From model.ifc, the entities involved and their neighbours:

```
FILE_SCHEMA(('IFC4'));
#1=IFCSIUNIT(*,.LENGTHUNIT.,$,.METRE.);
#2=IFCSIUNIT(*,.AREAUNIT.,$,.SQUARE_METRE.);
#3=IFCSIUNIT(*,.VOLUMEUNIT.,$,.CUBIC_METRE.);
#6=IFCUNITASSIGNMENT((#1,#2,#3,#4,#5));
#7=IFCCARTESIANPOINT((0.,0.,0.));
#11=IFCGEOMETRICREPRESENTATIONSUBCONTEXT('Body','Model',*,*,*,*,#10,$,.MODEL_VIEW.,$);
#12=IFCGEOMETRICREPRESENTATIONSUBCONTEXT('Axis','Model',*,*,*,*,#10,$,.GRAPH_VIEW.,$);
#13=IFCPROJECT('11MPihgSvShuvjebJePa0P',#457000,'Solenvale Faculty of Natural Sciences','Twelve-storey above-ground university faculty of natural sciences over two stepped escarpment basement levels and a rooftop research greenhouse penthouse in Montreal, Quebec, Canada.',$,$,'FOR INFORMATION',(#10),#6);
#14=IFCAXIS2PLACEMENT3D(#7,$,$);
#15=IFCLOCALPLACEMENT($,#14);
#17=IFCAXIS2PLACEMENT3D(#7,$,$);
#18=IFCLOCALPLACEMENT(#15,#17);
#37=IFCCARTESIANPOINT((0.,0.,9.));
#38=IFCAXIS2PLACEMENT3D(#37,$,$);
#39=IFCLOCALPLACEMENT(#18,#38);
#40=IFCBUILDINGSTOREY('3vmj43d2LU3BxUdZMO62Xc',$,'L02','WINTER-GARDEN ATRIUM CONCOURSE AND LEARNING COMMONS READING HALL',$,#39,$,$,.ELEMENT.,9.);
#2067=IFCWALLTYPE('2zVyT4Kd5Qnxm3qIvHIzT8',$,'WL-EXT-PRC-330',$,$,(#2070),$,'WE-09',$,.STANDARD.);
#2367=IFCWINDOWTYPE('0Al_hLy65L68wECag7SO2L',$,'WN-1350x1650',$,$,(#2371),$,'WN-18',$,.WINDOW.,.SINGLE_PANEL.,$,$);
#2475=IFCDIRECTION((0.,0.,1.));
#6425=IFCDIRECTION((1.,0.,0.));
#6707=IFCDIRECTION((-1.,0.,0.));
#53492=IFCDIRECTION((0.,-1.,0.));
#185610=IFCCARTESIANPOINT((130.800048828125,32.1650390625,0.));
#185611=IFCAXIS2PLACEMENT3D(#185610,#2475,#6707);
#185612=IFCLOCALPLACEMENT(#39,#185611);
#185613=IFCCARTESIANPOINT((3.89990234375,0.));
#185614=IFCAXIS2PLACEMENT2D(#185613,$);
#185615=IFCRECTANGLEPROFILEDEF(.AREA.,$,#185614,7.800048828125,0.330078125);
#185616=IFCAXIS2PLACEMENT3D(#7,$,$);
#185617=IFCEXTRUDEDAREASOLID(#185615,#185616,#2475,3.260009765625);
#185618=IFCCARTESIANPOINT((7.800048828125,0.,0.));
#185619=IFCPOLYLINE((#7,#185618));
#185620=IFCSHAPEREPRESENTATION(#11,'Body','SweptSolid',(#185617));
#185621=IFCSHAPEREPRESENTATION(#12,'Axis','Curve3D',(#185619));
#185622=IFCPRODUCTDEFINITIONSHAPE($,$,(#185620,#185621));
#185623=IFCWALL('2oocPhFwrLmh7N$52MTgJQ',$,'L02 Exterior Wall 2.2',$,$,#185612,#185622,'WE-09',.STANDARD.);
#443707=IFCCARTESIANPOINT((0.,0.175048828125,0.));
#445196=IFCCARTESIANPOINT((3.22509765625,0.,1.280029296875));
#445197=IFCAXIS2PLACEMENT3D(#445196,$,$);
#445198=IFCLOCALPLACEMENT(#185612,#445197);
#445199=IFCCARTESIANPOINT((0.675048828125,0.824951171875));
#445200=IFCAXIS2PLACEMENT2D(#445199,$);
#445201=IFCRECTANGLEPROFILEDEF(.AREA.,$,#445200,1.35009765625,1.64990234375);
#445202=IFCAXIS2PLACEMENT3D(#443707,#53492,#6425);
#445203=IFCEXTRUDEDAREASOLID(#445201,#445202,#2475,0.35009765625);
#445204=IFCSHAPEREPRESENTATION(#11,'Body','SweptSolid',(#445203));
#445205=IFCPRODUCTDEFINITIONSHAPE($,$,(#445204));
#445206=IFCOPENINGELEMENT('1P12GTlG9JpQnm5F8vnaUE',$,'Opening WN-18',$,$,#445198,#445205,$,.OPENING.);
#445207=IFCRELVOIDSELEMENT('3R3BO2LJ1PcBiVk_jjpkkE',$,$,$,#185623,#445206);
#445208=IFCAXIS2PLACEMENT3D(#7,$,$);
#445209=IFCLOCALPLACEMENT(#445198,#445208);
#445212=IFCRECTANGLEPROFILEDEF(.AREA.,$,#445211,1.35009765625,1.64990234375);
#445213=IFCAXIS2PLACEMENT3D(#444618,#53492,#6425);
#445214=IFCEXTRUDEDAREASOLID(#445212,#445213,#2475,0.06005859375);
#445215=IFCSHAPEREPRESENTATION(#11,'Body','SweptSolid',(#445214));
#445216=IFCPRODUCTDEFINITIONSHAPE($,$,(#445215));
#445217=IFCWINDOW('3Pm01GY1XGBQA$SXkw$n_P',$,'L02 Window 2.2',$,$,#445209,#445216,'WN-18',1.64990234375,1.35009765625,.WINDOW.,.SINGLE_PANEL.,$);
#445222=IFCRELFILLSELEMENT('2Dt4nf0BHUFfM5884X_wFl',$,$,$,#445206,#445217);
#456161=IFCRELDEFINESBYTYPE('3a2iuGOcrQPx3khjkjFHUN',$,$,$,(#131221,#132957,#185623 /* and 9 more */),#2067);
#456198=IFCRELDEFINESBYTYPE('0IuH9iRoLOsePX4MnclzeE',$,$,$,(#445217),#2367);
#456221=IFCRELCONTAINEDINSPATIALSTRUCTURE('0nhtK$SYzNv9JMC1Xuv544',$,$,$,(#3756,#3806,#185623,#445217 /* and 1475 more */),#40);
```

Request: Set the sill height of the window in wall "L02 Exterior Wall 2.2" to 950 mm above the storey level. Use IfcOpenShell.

```python
import numpy as np
import ifcopenshell
import ifcopenshell.api.geometry
import ifcopenshell.geom
import ifcopenshell.util.element
import ifcopenshell.util.placement
import ifcopenshell.util.shape
import ifcopenshell.util.unit

model = ifcopenshell.open("model.ifc")
unit_scale = ifcopenshell.util.unit.calculate_unit_scale(model)

window = model.by_guid("3Pm01GY1XGBQA$SXkw$n_P")
opening = window.FillsVoids[0].RelatingOpeningElement
storey = ifcopenshell.util.element.get_container(window, ifc_class="IfcBuildingStorey")
level = ifcopenshell.util.placement.get_local_placement(storey.ObjectPlacement)[2, 3]

# The opening's origin need not be at the sill, so measure its lowest point.
shape = ifcopenshell.geom.create_shape(ifcopenshell.geom.settings(), opening)
bottom = ifcopenshell.util.shape.get_shape_bottom_elevation(shape, shape.geometry) / unit_scale
dz = level + 0.95 / unit_scale - bottom

shift = np.array([0.0, 0.0, dz])
# The window is placed relative to its opening, so it follows when the opening moves.
matrix = ifcopenshell.util.placement.get_local_placement(opening.ObjectPlacement)
matrix[:3, 3] += shift
ifcopenshell.api.geometry.edit_object_placement(
    model, product=opening, matrix=matrix, is_si=False, should_transform_children=True
)

print(f"moved by {dz * unit_scale:+.3f} m")

model.write("model_edited.ifc")
```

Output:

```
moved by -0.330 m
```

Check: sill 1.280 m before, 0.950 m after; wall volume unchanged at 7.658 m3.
